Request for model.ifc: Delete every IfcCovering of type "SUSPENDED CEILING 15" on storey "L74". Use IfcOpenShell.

First a look at what the model holds.

```python
import ifcopenshell
import ifcopenshell.util.element

model = ifcopenshell.open("model.ifc")
print(model.schema)
storey = next(s for s in model.by_type("IfcBuildingStorey") if s.Name == "L74")
coverings = [e for e in ifcopenshell.util.element.get_decomposition(storey) if e.is_a("IfcCovering")]
seen = {}
for e in coverings:
    element_type = ifcopenshell.util.element.get_type(e)
    name = element_type.Name if element_type not in (None, e) else None
    seen[name] = seen.get(name, 0) + 1
for name, count in sorted(seen.items(), key=str):
    print(count, "x", name)
```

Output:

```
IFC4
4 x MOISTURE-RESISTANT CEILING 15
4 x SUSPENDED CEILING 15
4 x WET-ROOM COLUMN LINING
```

```python
import ifcopenshell
import ifcopenshell.api.root
import ifcopenshell.util.element

model = ifcopenshell.open("model.ifc")

storey = next(s for s in model.by_type("IfcBuildingStorey") if s.Name == "L74")
coverings = [e for e in ifcopenshell.util.element.get_decomposition(storey) if e.is_a("IfcCovering")]
targets = [e for e in coverings if (t := ifcopenshell.util.element.get_type(e)) not in (None, e) and t.Name == "SUSPENDED CEILING 15"]

for e in targets:
    ifcopenshell.api.root.remove_product(model, product=e)
print(len(targets), "removed")

model.write("model_updated.ifc")
```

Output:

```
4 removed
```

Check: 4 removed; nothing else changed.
